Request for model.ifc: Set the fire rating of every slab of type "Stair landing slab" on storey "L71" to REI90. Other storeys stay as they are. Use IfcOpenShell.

First a look at what the model holds.

```python
import ifcopenshell
import ifcopenshell.util.element

model = ifcopenshell.open("model.ifc")
print(model.schema)
storey = next(s for s in model.by_type("IfcBuildingStorey") if s.Name == "L71")
slabs = [e for e in ifcopenshell.util.element.get_decomposition(storey) if e.is_a("IfcSlab")]
seen = {}
for e in slabs:
    element_type = ifcopenshell.util.element.get_type(e)
    key = (element_type.Name if element_type != e and element_type else None, ifcopenshell.util.element.get_pset(e, "Pset_SlabCommon", "FireRating"))
    seen[key] = seen.get(key, 0) + 1
for (name, value), count in sorted(seen.items(), key=str):
    print(count, "x", name, "|", value)
```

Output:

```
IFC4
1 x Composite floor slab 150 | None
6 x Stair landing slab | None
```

```python
import ifcopenshell
import ifcopenshell.api.pset
import ifcopenshell.util.element

model = ifcopenshell.open("model.ifc")

storey = next(s for s in model.by_type("IfcBuildingStorey") if s.Name == "L71")
slabs = [e for e in ifcopenshell.util.element.get_decomposition(storey) if e.is_a("IfcSlab")]

count = 0
for e in slabs:
    element_type = ifcopenshell.util.element.get_type(e)
    if element_type in (None, e) or element_type.Name != "Stair landing slab":
        continue
    found = ifcopenshell.util.element.get_pset(e, "Pset_SlabCommon", should_inherit=False)
    if found:
        pset = model.by_id(found["id"])
        if len(ifcopenshell.util.element.get_elements_by_pset(pset)) > 1:
            pset = ifcopenshell.api.pset.unshare_pset(model, products=[e], pset=pset)[0]
    else:
        pset = ifcopenshell.api.pset.add_pset(model, product=e, name="Pset_SlabCommon")
    ifcopenshell.api.pset.edit_pset(model, pset=pset, properties={"FireRating": "REI90"})
    count += 1

print(count, "slabs updated")

model.write("model_v2.ifc")
```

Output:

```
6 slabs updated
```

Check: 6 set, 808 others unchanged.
